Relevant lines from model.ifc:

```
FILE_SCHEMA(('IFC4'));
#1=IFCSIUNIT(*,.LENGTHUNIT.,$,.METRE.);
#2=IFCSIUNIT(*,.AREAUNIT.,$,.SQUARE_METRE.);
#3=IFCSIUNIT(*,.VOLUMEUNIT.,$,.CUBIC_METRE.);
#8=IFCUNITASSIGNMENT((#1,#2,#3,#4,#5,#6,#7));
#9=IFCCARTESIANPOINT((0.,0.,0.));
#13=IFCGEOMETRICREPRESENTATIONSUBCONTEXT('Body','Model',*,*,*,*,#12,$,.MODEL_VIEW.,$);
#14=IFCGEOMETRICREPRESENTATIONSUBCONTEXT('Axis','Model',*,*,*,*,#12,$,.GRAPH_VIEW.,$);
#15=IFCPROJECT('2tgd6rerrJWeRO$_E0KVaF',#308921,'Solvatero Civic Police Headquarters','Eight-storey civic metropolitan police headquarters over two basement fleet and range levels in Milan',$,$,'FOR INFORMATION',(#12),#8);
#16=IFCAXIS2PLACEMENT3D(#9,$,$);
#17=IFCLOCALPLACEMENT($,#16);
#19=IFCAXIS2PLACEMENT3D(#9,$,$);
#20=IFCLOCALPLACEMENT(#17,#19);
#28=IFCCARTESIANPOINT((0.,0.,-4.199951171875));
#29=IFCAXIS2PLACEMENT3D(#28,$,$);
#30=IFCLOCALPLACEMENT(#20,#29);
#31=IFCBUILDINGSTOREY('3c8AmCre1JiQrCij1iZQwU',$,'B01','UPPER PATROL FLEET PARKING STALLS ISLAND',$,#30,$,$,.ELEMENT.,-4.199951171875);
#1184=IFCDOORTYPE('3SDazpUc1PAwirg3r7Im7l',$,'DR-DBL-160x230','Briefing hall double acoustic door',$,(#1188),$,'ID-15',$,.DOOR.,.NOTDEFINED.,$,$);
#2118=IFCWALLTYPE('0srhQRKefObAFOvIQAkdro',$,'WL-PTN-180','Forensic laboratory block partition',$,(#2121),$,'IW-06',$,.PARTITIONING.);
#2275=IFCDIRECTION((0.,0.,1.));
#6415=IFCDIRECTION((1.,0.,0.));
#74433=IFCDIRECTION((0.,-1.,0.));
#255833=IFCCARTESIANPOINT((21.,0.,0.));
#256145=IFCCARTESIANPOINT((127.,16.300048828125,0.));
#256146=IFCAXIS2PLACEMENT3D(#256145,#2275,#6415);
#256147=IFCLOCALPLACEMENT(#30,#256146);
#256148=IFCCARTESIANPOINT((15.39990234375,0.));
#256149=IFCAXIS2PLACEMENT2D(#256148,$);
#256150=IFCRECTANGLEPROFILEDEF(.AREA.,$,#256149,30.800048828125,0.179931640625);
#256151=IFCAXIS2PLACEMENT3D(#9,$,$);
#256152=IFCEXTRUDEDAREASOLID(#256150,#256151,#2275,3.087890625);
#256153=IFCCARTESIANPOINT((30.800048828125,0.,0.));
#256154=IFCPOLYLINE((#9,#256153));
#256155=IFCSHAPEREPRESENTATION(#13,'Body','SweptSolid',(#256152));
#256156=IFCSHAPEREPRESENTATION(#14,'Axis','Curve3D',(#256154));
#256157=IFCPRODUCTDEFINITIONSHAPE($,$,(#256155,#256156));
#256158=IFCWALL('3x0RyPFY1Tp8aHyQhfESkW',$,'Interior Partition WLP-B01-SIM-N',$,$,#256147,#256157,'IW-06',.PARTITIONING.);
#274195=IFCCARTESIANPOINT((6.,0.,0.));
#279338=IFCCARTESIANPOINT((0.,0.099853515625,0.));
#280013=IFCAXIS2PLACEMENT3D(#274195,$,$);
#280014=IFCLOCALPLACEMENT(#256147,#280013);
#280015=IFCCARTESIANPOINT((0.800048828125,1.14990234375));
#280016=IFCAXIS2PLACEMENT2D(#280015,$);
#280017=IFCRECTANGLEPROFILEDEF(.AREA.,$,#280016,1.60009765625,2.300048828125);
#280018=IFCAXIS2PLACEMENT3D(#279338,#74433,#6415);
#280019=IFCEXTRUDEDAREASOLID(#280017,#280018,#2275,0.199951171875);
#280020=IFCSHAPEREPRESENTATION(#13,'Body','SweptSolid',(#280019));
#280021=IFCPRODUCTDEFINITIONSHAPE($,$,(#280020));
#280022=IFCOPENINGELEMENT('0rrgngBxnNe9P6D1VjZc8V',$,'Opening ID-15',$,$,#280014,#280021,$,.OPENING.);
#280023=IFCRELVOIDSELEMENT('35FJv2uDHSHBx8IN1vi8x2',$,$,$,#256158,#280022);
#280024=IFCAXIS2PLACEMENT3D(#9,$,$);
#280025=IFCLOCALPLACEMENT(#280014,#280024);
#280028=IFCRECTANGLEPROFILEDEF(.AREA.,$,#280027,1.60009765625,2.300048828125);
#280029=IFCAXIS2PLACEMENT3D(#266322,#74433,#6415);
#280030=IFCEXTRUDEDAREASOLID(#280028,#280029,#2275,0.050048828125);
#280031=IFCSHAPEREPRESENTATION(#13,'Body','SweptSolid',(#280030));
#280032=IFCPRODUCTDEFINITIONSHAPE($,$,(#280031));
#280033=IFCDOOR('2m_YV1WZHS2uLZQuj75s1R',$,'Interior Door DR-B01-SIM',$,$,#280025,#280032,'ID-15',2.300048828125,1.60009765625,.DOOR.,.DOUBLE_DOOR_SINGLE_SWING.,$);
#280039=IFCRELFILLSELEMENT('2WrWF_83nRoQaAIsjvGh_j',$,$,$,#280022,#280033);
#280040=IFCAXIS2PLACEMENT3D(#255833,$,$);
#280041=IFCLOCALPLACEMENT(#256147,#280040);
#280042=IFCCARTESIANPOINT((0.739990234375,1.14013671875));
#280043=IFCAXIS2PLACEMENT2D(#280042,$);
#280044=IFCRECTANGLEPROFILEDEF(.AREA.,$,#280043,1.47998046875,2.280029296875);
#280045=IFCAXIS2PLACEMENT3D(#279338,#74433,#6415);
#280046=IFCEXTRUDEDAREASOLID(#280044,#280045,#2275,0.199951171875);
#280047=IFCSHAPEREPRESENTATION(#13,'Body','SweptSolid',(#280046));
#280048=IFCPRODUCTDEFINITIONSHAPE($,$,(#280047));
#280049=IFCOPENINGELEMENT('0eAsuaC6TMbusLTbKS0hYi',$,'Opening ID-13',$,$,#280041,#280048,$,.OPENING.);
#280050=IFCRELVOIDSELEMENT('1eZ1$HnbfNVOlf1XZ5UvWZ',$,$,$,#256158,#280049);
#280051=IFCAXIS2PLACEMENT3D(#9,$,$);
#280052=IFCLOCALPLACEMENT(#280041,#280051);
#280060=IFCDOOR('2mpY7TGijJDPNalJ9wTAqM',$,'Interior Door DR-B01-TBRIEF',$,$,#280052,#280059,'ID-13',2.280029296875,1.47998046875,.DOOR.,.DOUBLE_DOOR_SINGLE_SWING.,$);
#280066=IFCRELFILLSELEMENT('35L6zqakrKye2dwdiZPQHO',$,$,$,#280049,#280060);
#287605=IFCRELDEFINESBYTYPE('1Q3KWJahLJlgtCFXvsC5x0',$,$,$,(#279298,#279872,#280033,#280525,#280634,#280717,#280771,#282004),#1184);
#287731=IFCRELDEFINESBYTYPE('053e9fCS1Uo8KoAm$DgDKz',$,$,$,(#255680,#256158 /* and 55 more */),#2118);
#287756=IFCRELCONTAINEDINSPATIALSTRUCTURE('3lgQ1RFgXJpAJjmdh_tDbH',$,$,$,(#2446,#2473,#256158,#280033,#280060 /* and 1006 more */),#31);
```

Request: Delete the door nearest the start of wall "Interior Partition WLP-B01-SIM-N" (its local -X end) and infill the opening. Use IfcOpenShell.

```python
import ifcopenshell
import ifcopenshell.api.feature
import ifcopenshell.api.root
import ifcopenshell.geom
import ifcopenshell.util.shape

model = ifcopenshell.open("model.ifc")
settings = ifcopenshell.geom.settings()


def volume(element):
    """Net volume in cubic metres, openings subtracted."""
    shape = ifcopenshell.geom.create_shape(settings, element)
    return ifcopenshell.util.shape.get_volume(shape.geometry)


door = model.by_guid("2m_YV1WZHS2uLZQuj75s1R")
opening = door.FillsVoids[0].RelatingOpeningElement
wall = opening.VoidsElements[0].RelatingBuildingElement
before = volume(wall)

ifcopenshell.api.root.remove_product(model, product=door)
ifcopenshell.api.feature.remove_feature(model, feature=opening)

after = volume(wall)

print(f"wall volume {before:.3f} -> {after:.3f} m3")

model.write("model_edited.ifc")
```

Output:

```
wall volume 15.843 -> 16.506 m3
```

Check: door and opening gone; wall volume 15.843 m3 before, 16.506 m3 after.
